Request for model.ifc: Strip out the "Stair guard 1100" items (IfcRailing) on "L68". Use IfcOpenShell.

First a look at what the model holds.

```python
import ifcopenshell
import ifcopenshell.util.element

model = ifcopenshell.open("model.ifc")
print(model.schema)
storey = next(s for s in model.by_type("IfcBuildingStorey") if s.Name == "L68")
railings = [e for e in ifcopenshell.util.element.get_decomposition(storey) if e.is_a("IfcRailing")]
seen = {}
for e in railings:
    element_type = ifcopenshell.util.element.get_type(e)
    name = element_type.Name if element_type not in (None, e) else None
    seen[name] = seen.get(name, 0) + 1
for name, count in sorted(seen.items(), key=str):
    print(count, "x", name)
```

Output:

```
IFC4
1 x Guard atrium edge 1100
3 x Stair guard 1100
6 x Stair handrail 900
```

```python
import ifcopenshell
import ifcopenshell.api.root
import ifcopenshell.util.element

model = ifcopenshell.open("model.ifc")

storey = next(s for s in model.by_type("IfcBuildingStorey") if s.Name == "L68")
railings = [e for e in ifcopenshell.util.element.get_decomposition(storey) if e.is_a("IfcRailing")]
targets = [e for e in railings if (t := ifcopenshell.util.element.get_type(e)) not in (None, e) and t.Name == "Stair guard 1100"]

for e in targets:
    ifcopenshell.api.root.remove_product(model, product=e)
print(len(targets), "removed")

model.write("model_edited.ifc")
```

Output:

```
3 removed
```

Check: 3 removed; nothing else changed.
